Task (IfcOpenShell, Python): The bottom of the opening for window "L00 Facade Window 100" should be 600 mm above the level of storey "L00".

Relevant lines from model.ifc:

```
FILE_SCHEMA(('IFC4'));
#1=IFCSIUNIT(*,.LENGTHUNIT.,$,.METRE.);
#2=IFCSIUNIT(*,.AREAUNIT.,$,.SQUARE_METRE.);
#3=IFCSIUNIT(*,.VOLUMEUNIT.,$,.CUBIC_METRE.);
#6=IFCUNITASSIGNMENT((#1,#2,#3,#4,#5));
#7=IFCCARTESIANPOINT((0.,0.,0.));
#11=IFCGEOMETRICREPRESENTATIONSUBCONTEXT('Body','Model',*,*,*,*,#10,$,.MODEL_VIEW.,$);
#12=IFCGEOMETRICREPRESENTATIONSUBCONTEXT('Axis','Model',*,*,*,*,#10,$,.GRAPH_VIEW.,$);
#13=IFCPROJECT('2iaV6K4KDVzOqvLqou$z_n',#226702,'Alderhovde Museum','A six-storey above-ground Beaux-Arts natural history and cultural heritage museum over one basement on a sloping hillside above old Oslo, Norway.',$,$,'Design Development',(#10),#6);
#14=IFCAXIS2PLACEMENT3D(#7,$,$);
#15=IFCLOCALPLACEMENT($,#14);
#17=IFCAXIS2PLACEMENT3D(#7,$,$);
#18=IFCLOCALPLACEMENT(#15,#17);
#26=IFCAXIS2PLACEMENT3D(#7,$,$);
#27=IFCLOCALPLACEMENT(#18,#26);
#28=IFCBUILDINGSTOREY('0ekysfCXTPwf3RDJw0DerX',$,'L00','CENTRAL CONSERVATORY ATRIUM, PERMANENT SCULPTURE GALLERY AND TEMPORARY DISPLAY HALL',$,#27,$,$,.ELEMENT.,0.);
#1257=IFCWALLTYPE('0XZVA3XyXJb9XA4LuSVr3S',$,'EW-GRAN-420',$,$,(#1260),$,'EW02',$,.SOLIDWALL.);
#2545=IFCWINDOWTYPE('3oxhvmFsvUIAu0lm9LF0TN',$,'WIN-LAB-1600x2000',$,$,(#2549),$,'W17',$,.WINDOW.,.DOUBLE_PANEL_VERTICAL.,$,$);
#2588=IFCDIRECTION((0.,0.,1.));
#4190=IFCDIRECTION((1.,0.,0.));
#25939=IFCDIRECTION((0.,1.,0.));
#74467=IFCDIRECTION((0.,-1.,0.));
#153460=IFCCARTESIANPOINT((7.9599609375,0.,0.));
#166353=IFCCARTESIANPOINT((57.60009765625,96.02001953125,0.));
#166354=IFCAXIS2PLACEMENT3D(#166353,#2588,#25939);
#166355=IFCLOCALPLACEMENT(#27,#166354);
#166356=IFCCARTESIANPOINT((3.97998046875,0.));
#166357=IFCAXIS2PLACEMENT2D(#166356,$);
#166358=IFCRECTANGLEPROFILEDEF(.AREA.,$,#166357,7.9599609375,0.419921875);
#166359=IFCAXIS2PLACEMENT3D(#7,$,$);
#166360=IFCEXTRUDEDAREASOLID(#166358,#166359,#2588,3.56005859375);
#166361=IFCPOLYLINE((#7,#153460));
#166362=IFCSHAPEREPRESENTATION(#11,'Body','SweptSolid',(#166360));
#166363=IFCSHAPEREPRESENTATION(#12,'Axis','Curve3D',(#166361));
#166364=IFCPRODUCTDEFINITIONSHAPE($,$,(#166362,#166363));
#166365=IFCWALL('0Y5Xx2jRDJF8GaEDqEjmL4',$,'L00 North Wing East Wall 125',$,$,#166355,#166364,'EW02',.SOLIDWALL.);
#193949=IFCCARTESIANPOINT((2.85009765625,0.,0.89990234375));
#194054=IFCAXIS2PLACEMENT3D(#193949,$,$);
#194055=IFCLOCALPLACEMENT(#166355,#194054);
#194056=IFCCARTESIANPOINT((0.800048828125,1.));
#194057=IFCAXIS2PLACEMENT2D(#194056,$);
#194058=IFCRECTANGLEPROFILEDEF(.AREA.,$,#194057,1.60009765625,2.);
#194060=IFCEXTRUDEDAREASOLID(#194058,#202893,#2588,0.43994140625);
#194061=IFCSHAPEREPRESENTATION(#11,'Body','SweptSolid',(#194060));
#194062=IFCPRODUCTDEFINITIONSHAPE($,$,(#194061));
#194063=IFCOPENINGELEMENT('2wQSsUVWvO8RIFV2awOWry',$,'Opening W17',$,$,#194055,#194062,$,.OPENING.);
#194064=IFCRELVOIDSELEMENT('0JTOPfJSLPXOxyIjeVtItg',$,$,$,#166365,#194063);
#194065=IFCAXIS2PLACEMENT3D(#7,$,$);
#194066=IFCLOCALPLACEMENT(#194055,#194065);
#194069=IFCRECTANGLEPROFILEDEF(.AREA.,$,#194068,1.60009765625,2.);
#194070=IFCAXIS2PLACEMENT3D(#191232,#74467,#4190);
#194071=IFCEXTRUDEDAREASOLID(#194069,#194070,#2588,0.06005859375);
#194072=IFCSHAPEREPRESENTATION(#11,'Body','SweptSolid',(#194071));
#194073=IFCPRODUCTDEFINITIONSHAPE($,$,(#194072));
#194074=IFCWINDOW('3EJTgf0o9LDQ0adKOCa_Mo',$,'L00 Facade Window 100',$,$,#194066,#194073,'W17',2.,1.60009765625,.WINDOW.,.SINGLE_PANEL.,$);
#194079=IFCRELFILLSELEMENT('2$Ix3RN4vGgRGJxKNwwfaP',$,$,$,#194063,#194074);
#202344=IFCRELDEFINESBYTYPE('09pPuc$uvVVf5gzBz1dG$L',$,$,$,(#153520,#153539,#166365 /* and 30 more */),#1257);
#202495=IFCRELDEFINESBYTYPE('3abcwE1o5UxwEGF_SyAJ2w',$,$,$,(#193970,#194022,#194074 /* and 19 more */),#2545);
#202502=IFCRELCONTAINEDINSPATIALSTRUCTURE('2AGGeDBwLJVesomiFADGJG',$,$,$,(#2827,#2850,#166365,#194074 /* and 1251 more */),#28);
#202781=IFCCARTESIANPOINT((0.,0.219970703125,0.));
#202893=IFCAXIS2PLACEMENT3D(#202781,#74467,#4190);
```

```python
import numpy as np
import ifcopenshell
import ifcopenshell.api.geometry
import ifcopenshell.geom
import ifcopenshell.util.element
import ifcopenshell.util.placement
import ifcopenshell.util.shape
import ifcopenshell.util.unit

model = ifcopenshell.open("model.ifc")
unit_scale = ifcopenshell.util.unit.calculate_unit_scale(model)

window = model.by_guid("3EJTgf0o9LDQ0adKOCa_Mo")
opening = window.FillsVoids[0].RelatingOpeningElement
storey = ifcopenshell.util.element.get_container(window, ifc_class="IfcBuildingStorey")
level = ifcopenshell.util.placement.get_local_placement(storey.ObjectPlacement)[2, 3]

# The opening's origin need not be at the sill, so measure its lowest point.
shape = ifcopenshell.geom.create_shape(ifcopenshell.geom.settings(), opening)
bottom = ifcopenshell.util.shape.get_shape_bottom_elevation(shape, shape.geometry) / unit_scale
dz = level + 0.6 / unit_scale - bottom

shift = np.array([0.0, 0.0, dz])
# The window is placed relative to its opening, so it follows when the opening moves.
matrix = ifcopenshell.util.placement.get_local_placement(opening.ObjectPlacement)
matrix[:3, 3] += shift
ifcopenshell.api.geometry.edit_object_placement(
    model, product=opening, matrix=matrix, is_si=False, should_transform_children=True
)

print(f"moved by {dz * unit_scale:+.3f} m")

model.write("model-out.ifc")
```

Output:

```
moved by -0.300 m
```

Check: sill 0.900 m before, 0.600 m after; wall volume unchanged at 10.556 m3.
